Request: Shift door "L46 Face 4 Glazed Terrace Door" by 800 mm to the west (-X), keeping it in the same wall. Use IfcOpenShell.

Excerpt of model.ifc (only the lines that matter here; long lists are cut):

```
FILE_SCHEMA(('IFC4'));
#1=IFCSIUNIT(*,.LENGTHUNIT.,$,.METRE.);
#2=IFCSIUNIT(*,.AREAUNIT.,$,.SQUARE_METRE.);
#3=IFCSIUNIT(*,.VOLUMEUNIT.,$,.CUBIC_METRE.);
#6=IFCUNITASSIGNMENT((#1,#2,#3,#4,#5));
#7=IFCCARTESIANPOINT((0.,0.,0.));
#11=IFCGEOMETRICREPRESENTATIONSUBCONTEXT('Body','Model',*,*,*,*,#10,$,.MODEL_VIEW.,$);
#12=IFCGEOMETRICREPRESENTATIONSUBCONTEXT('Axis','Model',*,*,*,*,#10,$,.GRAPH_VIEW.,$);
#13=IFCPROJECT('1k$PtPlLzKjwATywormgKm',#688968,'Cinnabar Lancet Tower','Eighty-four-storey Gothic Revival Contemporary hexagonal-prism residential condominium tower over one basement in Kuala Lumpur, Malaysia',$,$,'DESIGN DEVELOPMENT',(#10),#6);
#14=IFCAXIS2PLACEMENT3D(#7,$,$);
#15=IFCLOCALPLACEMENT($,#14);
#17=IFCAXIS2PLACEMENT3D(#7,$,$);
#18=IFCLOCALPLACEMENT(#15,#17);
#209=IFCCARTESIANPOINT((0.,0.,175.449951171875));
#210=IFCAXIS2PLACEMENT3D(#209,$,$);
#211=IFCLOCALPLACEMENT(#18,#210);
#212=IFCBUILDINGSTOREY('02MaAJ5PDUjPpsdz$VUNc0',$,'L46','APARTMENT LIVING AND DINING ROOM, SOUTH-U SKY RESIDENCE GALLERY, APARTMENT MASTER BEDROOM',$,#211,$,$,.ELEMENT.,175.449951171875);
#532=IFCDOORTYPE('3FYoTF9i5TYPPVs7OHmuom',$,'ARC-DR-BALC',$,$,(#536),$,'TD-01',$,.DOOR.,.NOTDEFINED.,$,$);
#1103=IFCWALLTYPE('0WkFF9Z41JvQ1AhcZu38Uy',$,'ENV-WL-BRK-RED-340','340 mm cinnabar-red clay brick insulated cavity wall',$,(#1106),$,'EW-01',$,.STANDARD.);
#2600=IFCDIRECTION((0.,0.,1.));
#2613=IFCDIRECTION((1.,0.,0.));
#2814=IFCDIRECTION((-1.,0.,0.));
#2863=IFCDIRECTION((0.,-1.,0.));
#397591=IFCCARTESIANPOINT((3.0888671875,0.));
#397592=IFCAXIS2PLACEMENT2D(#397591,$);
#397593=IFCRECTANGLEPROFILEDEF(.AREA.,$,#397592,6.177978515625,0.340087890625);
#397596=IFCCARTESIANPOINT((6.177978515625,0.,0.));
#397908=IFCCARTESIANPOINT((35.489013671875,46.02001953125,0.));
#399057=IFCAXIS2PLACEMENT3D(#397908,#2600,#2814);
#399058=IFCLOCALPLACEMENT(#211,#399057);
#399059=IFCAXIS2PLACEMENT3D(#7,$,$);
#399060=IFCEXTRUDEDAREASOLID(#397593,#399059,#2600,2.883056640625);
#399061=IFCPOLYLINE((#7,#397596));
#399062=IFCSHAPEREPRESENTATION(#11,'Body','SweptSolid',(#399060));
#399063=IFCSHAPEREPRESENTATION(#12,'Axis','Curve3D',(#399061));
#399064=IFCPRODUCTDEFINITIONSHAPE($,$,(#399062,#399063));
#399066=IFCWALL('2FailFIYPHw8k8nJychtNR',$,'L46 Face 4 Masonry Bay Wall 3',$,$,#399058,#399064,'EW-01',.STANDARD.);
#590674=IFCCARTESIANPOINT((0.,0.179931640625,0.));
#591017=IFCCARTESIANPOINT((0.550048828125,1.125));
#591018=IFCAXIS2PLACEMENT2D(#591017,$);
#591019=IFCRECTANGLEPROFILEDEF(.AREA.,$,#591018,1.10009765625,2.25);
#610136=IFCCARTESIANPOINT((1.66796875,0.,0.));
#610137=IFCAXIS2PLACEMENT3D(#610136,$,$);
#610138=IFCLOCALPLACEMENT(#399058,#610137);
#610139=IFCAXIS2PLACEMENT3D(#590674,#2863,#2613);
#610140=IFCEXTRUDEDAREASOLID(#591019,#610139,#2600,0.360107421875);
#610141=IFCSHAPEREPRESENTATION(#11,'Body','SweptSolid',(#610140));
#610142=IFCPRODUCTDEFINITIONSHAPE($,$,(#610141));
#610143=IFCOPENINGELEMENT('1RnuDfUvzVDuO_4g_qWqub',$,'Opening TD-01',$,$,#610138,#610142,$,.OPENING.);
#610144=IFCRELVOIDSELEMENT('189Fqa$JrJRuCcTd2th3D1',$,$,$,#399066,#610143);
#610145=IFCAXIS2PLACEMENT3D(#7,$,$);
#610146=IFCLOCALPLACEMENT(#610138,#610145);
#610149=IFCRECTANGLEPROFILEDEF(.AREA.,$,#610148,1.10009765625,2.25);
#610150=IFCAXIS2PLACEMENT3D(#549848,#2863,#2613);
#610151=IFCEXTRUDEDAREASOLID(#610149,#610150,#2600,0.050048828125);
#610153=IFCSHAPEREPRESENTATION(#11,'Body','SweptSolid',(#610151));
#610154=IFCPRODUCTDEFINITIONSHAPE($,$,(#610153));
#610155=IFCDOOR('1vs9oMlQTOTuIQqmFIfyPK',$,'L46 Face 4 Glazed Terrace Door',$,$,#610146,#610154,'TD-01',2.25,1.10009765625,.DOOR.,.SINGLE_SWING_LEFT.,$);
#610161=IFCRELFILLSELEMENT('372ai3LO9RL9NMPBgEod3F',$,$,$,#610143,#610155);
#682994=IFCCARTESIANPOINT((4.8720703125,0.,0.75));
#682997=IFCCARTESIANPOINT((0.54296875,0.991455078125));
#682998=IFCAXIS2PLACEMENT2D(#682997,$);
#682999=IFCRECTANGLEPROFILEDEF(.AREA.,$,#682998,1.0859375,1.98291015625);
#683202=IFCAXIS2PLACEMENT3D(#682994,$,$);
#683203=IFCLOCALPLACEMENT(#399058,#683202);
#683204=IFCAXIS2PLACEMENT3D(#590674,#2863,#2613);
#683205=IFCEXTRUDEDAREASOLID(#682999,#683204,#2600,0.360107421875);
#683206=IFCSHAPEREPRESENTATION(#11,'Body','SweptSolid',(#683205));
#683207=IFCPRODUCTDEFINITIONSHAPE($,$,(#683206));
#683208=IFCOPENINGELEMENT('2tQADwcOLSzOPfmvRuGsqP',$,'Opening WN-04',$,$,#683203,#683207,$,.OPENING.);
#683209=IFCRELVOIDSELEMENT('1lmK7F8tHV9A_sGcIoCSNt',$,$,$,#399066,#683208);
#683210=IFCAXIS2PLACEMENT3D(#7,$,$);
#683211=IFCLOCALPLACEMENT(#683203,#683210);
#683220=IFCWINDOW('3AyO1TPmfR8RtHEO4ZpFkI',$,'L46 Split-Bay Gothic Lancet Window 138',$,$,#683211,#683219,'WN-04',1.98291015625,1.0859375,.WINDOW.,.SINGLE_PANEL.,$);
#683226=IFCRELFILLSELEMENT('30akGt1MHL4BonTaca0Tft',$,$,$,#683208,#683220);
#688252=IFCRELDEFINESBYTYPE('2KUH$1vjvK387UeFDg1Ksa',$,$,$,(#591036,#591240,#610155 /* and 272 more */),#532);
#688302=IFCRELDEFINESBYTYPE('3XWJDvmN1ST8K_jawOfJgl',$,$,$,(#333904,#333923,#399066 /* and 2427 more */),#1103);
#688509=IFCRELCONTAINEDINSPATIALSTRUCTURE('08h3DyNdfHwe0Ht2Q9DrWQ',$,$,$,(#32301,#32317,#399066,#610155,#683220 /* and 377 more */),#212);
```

```python
import ifcopenshell
import ifcopenshell.api.geometry
import ifcopenshell.util.placement
import ifcopenshell.util.unit

model = ifcopenshell.open("model.ifc")
unit_scale = ifcopenshell.util.unit.calculate_unit_scale(model)

door = model.by_guid("1vs9oMlQTOTuIQqmFIfyPK")
opening = door.FillsVoids[0].RelatingOpeningElement
wall = opening.VoidsElements[0].RelatingBuildingElement

wall_matrix = ifcopenshell.util.placement.get_local_placement(wall.ObjectPlacement)
shift = wall_matrix[:3, 0] * 0.8 / unit_scale
before = ifcopenshell.util.placement.get_local_placement(door.ObjectPlacement)[:3, 3].copy()

# The door is placed relative to its opening, so it follows when the opening moves.
matrix = ifcopenshell.util.placement.get_local_placement(opening.ObjectPlacement)
matrix[:3, 3] += shift
ifcopenshell.api.geometry.edit_object_placement(
    model, product=opening, matrix=matrix, is_si=False, should_transform_children=True
)

after = ifcopenshell.util.placement.get_local_placement(door.ObjectPlacement)[:3, 3]
print("door moved by", (after - before).round(3) + 0.0)

model.write("model-out.ifc")
```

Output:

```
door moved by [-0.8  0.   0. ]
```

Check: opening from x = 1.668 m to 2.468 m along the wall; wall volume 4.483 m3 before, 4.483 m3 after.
